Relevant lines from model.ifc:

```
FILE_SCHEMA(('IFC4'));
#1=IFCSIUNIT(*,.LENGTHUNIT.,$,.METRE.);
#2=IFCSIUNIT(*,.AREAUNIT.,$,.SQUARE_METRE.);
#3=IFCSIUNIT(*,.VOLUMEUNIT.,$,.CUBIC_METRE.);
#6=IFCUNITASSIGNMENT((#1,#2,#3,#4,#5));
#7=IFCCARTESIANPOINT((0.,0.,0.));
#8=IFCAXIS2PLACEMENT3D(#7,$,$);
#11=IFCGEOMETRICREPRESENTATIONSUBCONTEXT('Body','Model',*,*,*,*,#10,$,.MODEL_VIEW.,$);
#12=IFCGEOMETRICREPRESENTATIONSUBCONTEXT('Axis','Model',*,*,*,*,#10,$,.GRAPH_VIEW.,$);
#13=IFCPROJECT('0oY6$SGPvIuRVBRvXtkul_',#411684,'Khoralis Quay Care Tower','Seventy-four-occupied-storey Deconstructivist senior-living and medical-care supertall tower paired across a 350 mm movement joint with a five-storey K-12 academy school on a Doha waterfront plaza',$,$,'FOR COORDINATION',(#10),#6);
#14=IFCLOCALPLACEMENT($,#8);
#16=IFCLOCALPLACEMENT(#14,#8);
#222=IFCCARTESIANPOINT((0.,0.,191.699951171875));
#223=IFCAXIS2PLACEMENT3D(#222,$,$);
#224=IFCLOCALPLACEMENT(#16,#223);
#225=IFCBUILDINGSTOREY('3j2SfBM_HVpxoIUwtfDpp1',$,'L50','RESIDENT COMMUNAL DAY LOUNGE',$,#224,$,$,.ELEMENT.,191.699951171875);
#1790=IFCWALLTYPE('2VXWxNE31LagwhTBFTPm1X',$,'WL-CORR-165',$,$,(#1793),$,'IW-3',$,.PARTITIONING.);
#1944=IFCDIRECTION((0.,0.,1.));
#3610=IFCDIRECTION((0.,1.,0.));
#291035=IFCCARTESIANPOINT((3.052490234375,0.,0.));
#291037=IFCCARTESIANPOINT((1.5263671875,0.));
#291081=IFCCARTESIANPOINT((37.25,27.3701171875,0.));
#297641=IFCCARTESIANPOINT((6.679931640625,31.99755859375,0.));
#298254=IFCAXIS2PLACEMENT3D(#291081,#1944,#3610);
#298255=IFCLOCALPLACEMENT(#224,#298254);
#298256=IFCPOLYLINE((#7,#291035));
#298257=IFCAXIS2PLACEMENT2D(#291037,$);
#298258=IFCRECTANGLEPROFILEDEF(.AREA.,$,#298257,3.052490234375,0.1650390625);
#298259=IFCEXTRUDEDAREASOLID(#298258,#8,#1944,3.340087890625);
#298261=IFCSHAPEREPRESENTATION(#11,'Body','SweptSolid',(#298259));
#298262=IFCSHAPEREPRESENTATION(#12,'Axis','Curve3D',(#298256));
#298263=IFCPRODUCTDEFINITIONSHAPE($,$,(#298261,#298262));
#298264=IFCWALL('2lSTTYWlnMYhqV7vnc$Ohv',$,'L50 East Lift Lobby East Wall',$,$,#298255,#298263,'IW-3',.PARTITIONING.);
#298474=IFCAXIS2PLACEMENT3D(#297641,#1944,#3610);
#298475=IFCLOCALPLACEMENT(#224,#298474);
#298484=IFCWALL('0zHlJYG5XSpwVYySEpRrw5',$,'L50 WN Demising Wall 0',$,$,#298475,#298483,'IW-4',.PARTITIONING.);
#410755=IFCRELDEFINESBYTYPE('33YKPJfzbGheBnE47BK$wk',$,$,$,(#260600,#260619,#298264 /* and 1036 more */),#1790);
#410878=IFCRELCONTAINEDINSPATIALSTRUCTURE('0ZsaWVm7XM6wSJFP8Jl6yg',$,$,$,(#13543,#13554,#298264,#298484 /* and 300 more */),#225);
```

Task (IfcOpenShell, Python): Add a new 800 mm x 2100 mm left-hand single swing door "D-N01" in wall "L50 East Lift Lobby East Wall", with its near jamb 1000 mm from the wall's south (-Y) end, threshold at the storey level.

```python
import numpy as np
import ifcopenshell
import ifcopenshell.api.feature
import ifcopenshell.api.geometry
import ifcopenshell.api.root
import ifcopenshell.api.spatial
import ifcopenshell.geom
import ifcopenshell.util.element
import ifcopenshell.util.placement
import ifcopenshell.util.representation
import ifcopenshell.util.shape
import ifcopenshell.util.unit

model = ifcopenshell.open("model.ifc")
unit_scale = ifcopenshell.util.unit.calculate_unit_scale(model)
settings = ifcopenshell.geom.settings()


def volume(element):
    """Net volume in cubic metres, openings subtracted."""
    shape = ifcopenshell.geom.create_shape(settings, element)
    return ifcopenshell.util.shape.get_volume(shape.geometry)


wall = model.by_guid("2lSTTYWlnMYhqV7vnc$Ohv")
storey = ifcopenshell.util.element.get_container(wall, ifc_class="IfcBuildingStorey")
context = ifcopenshell.util.representation.get_context(model, "Model", "Body", "MODEL_VIEW")
before = volume(wall)

width, height, from_end, sill = 0.8, 2.1, 1, 0.0  # metres

# The wall runs along its own X axis, and the end named is its -X end.
wall_shape = ifcopenshell.geom.create_shape(settings, wall)
x, y, z = ifcopenshell.util.shape.get_vertices(wall_shape.geometry).T
start = x.min() + from_end
face, thickness = float(y.min()), float(y.max() - y.min())
wall_matrix = ifcopenshell.util.placement.get_local_placement(wall.ObjectPlacement)
level = ifcopenshell.util.placement.get_local_placement(storey.ObjectPlacement)[2, 3]


def in_wall(x, y):
    """Placement at x, y metres in the wall's axes, at sill height."""
    matrix = wall_matrix.copy()
    matrix[:, 3] = wall_matrix @ np.array([x / unit_scale, y / unit_scale, 0.0, 1.0])
    matrix[2, 3] = level + sill / unit_scale
    return matrix


# Opening: a box that overshoots both wall faces by 50 mm.
opening = ifcopenshell.api.root.create_entity(model, ifc_class="IfcOpeningElement", predefined_type="OPENING")
box = ifcopenshell.api.geometry.add_wall_representation(
    model, context=context, length=width, height=height, thickness=thickness + 0.1
)
ifcopenshell.api.geometry.assign_representation(model, product=opening, representation=box)
ifcopenshell.api.geometry.edit_object_placement(model, product=opening, matrix=in_wall(start, face - 0.05), is_si=False)
ifcopenshell.api.feature.add_feature(model, feature=opening, element=wall)

door = ifcopenshell.api.root.create_entity(model, ifc_class="IfcDoor", name="D-N01", predefined_type="DOOR")
door.OverallWidth, door.OverallHeight = width / unit_scale, height / unit_scale
door.OperationType = "SINGLE_SWING_LEFT"
body = ifcopenshell.api.geometry.add_door_representation(
    model,
    context=context,
    overall_width=door.OverallWidth,
    overall_height=door.OverallHeight,
    operation_type="SINGLE_SWING_LEFT",
    lining_properties={"LiningDepth": thickness / unit_scale, "ThresholdDepth": thickness / unit_scale},
)
ifcopenshell.api.geometry.assign_representation(model, product=door, representation=body)
ifcopenshell.api.spatial.assign_container(model, products=[door], relating_structure=storey)
ifcopenshell.api.feature.add_filling(model, opening=opening, element=door)

# The lining spans the wall, so the door starts at the wall face.
ifcopenshell.api.geometry.edit_object_placement(model, product=door, matrix=in_wall(start, face), is_si=False)

after = volume(wall)

print(f"wall volume {before:.3f} -> {after:.3f} m3")

model.write("model-out.ifc")
```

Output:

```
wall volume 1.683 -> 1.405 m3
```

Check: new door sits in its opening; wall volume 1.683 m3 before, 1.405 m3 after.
